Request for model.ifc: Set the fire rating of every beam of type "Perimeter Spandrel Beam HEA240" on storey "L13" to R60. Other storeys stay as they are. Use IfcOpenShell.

First a look at what the model holds.

```python
import ifcopenshell
import ifcopenshell.util.element

model = ifcopenshell.open("model.ifc")
print(model.schema)
storey = next(s for s in model.by_type("IfcBuildingStorey") if s.Name == "L13")
beams = [e for e in ifcopenshell.util.element.get_decomposition(storey) if e.is_a("IfcBeam")]
seen = {}
for e in beams:
    element_type = ifcopenshell.util.element.get_type(e)
    key = (element_type.Name if element_type != e and element_type else None, ifcopenshell.util.element.get_pset(e, "Pset_BeamCommon", "FireRating"))
    seen[key] = seen.get(key, 0) + 1
for (name, value), count in sorted(seen.items(), key=str):
    print(count, "x", name, "|", value)
```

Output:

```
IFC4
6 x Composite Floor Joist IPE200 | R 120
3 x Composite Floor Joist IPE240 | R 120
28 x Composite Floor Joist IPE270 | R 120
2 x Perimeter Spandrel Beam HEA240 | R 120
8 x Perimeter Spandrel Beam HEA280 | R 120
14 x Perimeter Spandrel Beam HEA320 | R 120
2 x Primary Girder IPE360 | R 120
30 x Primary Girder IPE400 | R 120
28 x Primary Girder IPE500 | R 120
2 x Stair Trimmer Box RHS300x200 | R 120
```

```python
import ifcopenshell
import ifcopenshell.api.pset
import ifcopenshell.util.element

model = ifcopenshell.open("model.ifc")

storey = next(s for s in model.by_type("IfcBuildingStorey") if s.Name == "L13")
beams = [e for e in ifcopenshell.util.element.get_decomposition(storey) if e.is_a("IfcBeam")]

count = 0
for e in beams:
    element_type = ifcopenshell.util.element.get_type(e)
    if element_type in (None, e) or element_type.Name != "Perimeter Spandrel Beam HEA240":
        continue
    # add_pset returns the element's existing set when there is one.
    pset = ifcopenshell.api.pset.add_pset(model, product=e, name="Pset_BeamCommon")
    ifcopenshell.api.pset.edit_pset(model, pset=pset, properties={"FireRating": "R60"})
    count += 1

print(count, "beams updated")

model.write("model-out.ifc")
```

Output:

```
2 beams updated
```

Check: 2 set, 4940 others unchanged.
